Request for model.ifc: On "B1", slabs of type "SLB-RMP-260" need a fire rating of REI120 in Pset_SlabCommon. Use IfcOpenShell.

First a look at what the model holds.

```python
import ifcopenshell
import ifcopenshell.util.element

model = ifcopenshell.open("model.ifc")
print(model.schema)
storey = next(s for s in model.by_type("IfcBuildingStorey") if s.Name == "B1")
slabs = [e for e in ifcopenshell.util.element.get_decomposition(storey) if e.is_a("IfcSlab")]
seen = {}
for e in slabs:
    element_type = ifcopenshell.util.element.get_type(e)
    key = (element_type.Name if element_type != e and element_type else None, ifcopenshell.util.element.get_pset(e, "Pset_SlabCommon", "FireRating"))
    seen[key] = seen.get(key, 0) + 1
for (name, value), count in sorted(seen.items(), key=str):
    print(count, "x", name, "|", value)
```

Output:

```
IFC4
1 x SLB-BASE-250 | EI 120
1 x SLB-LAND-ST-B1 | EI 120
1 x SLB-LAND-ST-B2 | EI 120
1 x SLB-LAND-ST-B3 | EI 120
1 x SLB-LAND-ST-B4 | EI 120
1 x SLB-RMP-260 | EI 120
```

```python
import ifcopenshell
import ifcopenshell.api.pset
import ifcopenshell.util.element

model = ifcopenshell.open("model.ifc")

storey = next(s for s in model.by_type("IfcBuildingStorey") if s.Name == "B1")
slabs = [e for e in ifcopenshell.util.element.get_decomposition(storey) if e.is_a("IfcSlab")]

count = 0
for e in slabs:
    element_type = ifcopenshell.util.element.get_type(e)
    if element_type in (None, e) or element_type.Name != "SLB-RMP-260":
        continue
    # add_pset returns the element's existing set when there is one.
    pset = ifcopenshell.api.pset.add_pset(model, product=e, name="Pset_SlabCommon")
    ifcopenshell.api.pset.edit_pset(model, pset=pset, properties={"FireRating": "REI120"})
    count += 1

print(count, "slabs updated")

model.write("model_v2.ifc")
```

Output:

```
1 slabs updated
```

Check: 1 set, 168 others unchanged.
